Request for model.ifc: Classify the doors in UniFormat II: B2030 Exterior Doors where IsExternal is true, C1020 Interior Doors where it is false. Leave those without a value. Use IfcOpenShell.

First a look at what the model holds.

```python
import ifcopenshell
import ifcopenshell.util.element

model = ifcopenshell.open("model.ifc")
print(model.schema)
print("classifications:", [c.Name for c in model.by_type("IfcClassification")])
values = [ifcopenshell.util.element.get_pset(e, "Pset_DoorCommon", "IsExternal") for e in model.by_type("IfcDoor")]
for value in (True, False, None):
    print("IsExternal", value, values.count(value))
```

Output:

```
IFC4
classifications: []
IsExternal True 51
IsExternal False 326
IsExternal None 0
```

```python
import ifcopenshell
import ifcopenshell.api.classification
import ifcopenshell.util.element

model = ifcopenshell.open("model.ifc")

system = ifcopenshell.api.classification.add_classification(model, classification="UniFormat II")

doors = model.by_type("IfcDoor")
external = {e: ifcopenshell.util.element.get_pset(e, "Pset_DoorCommon", "IsExternal") for e in doors}
for flag, code, name in ((True, "B2030", "Exterior Doors"), (False, "C1020", "Interior Doors")):
    products = [e for e in doors if external[e] is flag]
    ifcopenshell.api.classification.add_reference(
        model, products=products, classification=system, identification=code, name=name
    )
    print(code, len(products))

model.write("model_edited.ifc")
```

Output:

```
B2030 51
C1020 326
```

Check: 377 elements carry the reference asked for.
